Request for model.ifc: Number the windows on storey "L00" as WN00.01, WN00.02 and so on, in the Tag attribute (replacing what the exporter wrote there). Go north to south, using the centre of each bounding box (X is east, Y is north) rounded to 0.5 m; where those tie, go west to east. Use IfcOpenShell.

First a look at what the model holds.

```python
import ifcopenshell
import ifcopenshell.util.element
import ifcopenshell.util.placement

model = ifcopenshell.open("model.ifc")
print(model.schema)
storey = next(s for s in model.by_type("IfcBuildingStorey") if s.Name == "L00")
windows = [e for e in ifcopenshell.util.element.get_decomposition(storey) if e.is_a("IfcWindow")]
for e in sorted(windows, key=lambda e: e.id()):
    origin = ifcopenshell.util.placement.get_local_placement(e.ObjectPlacement)[:3, 3]
    print(e.id(), e.Tag, e.Name, origin.round(2) + 0.0, sep=" | ")
```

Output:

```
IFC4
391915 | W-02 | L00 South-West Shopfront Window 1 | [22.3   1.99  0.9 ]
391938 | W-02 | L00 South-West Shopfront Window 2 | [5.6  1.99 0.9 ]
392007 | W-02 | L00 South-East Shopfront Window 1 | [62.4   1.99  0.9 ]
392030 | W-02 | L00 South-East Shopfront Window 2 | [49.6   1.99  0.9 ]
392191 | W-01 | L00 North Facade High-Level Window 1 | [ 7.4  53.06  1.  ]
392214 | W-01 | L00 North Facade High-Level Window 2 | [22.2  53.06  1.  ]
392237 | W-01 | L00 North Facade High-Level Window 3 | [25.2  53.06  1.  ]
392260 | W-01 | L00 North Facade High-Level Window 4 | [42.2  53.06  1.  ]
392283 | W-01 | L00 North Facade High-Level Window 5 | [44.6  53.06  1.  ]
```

```python
import ifcopenshell
import ifcopenshell.geom
import ifcopenshell.util.element
import ifcopenshell.util.shape

model = ifcopenshell.open("model.ifc")
settings = ifcopenshell.geom.settings()
settings.set("use-world-coords", True)


def centre(element):
    shape = ifcopenshell.geom.create_shape(settings, element)
    return ifcopenshell.util.shape.get_bbox_centroid(shape.geometry)


storey = next(s for s in model.by_type("IfcBuildingStorey") if s.Name == "L00")
windows = [e for e in ifcopenshell.util.element.get_decomposition(storey) if e.is_a("IfcWindow")]

# Insertion points can sit at a corner or the storey origin, so sort by the geometry (in metres).
centres = {e: centre(e) for e in windows}
windows.sort(key=lambda e: (-round(centres[e][1] / 0.5), centres[e][0]))

for i, e in enumerate(windows, start=1):
    number = f"WN00.{i:02d}"
    e.Tag = number
    print(e.id(), number)

model.write("model_edited.ifc")
```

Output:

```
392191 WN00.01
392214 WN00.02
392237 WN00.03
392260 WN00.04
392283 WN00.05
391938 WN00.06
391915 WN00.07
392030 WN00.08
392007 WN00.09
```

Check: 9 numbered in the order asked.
